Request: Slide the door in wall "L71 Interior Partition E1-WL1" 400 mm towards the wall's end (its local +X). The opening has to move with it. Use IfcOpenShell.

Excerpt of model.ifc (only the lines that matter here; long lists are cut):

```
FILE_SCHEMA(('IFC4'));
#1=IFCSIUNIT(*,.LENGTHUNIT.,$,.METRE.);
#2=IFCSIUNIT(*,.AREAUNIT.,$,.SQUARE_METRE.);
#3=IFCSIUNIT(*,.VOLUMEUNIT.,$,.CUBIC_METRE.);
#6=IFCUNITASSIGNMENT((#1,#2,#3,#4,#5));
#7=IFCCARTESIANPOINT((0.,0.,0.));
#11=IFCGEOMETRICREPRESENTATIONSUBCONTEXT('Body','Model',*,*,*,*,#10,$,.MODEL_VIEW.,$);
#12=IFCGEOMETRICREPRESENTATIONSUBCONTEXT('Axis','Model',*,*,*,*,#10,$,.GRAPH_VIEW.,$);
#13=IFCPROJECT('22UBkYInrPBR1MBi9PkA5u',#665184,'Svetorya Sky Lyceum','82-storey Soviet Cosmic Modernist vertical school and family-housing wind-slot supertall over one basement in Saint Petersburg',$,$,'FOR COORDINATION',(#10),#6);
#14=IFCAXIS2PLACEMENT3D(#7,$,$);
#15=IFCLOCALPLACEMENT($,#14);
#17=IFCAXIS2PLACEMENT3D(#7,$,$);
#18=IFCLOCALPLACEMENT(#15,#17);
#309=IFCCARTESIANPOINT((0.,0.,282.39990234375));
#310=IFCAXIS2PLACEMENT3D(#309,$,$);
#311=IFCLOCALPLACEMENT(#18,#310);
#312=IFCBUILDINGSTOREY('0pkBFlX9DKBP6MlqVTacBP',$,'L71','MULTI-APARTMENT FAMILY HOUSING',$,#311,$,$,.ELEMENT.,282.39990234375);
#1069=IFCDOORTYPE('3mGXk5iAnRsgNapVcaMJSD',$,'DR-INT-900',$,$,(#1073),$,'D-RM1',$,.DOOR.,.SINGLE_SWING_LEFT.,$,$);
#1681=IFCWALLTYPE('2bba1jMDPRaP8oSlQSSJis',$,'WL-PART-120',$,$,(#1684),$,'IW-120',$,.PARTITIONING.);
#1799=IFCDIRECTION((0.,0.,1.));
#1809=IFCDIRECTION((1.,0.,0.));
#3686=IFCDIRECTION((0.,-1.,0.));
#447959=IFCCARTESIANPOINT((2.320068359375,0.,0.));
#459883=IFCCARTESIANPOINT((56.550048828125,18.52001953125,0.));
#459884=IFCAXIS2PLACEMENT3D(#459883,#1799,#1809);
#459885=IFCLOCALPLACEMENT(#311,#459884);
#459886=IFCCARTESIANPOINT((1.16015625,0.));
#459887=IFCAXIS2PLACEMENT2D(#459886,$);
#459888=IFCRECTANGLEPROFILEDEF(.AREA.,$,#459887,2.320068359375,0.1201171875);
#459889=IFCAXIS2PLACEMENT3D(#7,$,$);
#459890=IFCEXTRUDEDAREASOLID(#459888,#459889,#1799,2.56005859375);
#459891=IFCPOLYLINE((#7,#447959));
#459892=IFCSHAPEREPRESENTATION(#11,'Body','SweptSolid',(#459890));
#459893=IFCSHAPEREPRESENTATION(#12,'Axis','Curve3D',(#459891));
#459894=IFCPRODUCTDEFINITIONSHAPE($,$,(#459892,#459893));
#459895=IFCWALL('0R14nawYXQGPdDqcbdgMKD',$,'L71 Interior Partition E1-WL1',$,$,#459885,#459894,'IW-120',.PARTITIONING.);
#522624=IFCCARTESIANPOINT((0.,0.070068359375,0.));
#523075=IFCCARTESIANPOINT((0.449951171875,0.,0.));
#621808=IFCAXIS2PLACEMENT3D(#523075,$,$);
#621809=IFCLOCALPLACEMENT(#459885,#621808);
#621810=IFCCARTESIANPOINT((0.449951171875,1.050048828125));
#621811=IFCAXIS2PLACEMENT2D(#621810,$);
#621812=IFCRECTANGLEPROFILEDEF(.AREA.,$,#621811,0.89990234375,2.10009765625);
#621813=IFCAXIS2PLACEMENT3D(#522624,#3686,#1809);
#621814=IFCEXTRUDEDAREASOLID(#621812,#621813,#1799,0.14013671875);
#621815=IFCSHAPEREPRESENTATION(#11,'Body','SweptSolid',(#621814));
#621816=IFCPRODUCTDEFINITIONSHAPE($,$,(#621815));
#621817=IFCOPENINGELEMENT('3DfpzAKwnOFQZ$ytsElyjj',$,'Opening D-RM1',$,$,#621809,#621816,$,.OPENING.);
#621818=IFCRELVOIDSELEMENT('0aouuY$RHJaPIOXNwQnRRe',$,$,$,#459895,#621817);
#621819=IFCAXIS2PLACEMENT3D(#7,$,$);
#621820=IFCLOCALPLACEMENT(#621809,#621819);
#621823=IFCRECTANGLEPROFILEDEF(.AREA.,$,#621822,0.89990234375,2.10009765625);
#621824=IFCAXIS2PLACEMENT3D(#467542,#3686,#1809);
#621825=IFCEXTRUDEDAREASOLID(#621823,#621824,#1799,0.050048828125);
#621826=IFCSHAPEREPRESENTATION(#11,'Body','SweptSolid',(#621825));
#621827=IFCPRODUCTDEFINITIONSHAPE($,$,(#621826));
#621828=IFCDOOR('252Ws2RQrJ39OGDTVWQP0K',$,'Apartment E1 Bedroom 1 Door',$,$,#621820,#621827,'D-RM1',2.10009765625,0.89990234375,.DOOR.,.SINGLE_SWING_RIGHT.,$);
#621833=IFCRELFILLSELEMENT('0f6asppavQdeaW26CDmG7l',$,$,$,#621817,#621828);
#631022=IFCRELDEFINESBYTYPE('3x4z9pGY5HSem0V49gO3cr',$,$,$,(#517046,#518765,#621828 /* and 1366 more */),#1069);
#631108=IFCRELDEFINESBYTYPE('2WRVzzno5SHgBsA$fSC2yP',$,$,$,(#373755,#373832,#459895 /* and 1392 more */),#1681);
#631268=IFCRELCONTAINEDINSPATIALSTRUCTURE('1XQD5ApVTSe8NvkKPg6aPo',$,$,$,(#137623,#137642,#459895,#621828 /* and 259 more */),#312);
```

```python
import ifcopenshell
import ifcopenshell.api.geometry
import ifcopenshell.util.placement

model = ifcopenshell.open("model.ifc")

door = model.by_id(621828)
opening = door.FillsVoids[0].RelatingOpeningElement
wall = opening.VoidsElements[0].RelatingBuildingElement

wall_matrix = ifcopenshell.util.placement.get_local_placement(wall.ObjectPlacement)
shift = wall_matrix[:3, 0] * 0.4
before = ifcopenshell.util.placement.get_local_placement(door.ObjectPlacement)[:3, 3].copy()

# The door is placed relative to its opening, so it follows when the opening moves.
matrix = ifcopenshell.util.placement.get_local_placement(opening.ObjectPlacement)
matrix[:3, 3] += shift
ifcopenshell.api.geometry.edit_object_placement(
    model, product=opening, matrix=matrix, is_si=False, should_transform_children=True
)

after = ifcopenshell.util.placement.get_local_placement(door.ObjectPlacement)[:3, 3]
print("door moved by", (after - before).round(3) + 0.0)

model.write("model-out.ifc")
```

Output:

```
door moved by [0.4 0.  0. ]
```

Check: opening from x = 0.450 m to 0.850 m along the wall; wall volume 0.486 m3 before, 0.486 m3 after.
